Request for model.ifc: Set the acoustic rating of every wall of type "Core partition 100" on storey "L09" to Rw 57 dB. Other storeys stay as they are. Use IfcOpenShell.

First a look at what the model holds.

```python
import ifcopenshell
import ifcopenshell.util.element

model = ifcopenshell.open("model.ifc")
print(model.schema)
storey = next(s for s in model.by_type("IfcBuildingStorey") if s.Name == "L09")
walls = [e for e in ifcopenshell.util.element.get_decomposition(storey) if e.is_a("IfcWall")]
seen = {}
for e in walls:
    element_type = ifcopenshell.util.element.get_type(e)
    key = (element_type.Name if element_type != e and element_type else None, ifcopenshell.util.element.get_pset(e, "Pset_WallCommon", "AcousticRating"))
    seen[key] = seen.get(key, 0) + 1
for (name, value), count in sorted(seen.items(), key=str):
    print(count, "x", name, "|", value)
```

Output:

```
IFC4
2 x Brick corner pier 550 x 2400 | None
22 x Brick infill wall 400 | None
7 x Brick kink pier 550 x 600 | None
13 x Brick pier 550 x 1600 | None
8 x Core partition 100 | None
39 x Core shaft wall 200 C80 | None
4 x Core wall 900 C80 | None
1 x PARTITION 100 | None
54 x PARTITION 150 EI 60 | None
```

```python
import ifcopenshell
import ifcopenshell.api.pset
import ifcopenshell.util.element

model = ifcopenshell.open("model.ifc")

storey = next(s for s in model.by_type("IfcBuildingStorey") if s.Name == "L09")
walls = [e for e in ifcopenshell.util.element.get_decomposition(storey) if e.is_a("IfcWall")]

count = 0
for e in walls:
    element_type = ifcopenshell.util.element.get_type(e)
    if element_type in (None, e) or element_type.Name != "Core partition 100":
        continue
    found = ifcopenshell.util.element.get_pset(e, "Pset_WallCommon", should_inherit=False)
    if found:
        pset = model.by_id(found["id"])
        if len(ifcopenshell.util.element.get_elements_by_pset(pset)) > 1:
            pset = ifcopenshell.api.pset.unshare_pset(model, products=[e], pset=pset)[0]
    else:
        pset = ifcopenshell.api.pset.add_pset(model, product=e, name="Pset_WallCommon")
    ifcopenshell.api.pset.edit_pset(model, pset=pset, properties={"AcousticRating": "Rw 57 dB"})
    count += 1

print(count, "walls updated")

model.write("model-out.ifc")
```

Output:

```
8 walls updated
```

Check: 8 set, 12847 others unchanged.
